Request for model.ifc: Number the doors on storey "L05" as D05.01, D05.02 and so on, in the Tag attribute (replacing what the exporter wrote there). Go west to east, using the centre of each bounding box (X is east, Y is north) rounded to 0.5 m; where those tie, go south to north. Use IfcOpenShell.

First a look at what the model holds.

```python
import ifcopenshell
import ifcopenshell.util.element
import ifcopenshell.util.placement

model = ifcopenshell.open("model.ifc")
print(model.schema)
storey = next(s for s in model.by_type("IfcBuildingStorey") if s.Name == "L05")
doors = [e for e in ifcopenshell.util.element.get_decomposition(storey) if e.is_a("IfcDoor")]
for e in sorted(doors, key=lambda e: e.id()):
    origin = ifcopenshell.util.placement.get_local_placement(e.ObjectPlacement)[:3, 3]
    print(e.id(), e.Tag, e.Name, origin.round(2) + 0.0, sep=" | ")
```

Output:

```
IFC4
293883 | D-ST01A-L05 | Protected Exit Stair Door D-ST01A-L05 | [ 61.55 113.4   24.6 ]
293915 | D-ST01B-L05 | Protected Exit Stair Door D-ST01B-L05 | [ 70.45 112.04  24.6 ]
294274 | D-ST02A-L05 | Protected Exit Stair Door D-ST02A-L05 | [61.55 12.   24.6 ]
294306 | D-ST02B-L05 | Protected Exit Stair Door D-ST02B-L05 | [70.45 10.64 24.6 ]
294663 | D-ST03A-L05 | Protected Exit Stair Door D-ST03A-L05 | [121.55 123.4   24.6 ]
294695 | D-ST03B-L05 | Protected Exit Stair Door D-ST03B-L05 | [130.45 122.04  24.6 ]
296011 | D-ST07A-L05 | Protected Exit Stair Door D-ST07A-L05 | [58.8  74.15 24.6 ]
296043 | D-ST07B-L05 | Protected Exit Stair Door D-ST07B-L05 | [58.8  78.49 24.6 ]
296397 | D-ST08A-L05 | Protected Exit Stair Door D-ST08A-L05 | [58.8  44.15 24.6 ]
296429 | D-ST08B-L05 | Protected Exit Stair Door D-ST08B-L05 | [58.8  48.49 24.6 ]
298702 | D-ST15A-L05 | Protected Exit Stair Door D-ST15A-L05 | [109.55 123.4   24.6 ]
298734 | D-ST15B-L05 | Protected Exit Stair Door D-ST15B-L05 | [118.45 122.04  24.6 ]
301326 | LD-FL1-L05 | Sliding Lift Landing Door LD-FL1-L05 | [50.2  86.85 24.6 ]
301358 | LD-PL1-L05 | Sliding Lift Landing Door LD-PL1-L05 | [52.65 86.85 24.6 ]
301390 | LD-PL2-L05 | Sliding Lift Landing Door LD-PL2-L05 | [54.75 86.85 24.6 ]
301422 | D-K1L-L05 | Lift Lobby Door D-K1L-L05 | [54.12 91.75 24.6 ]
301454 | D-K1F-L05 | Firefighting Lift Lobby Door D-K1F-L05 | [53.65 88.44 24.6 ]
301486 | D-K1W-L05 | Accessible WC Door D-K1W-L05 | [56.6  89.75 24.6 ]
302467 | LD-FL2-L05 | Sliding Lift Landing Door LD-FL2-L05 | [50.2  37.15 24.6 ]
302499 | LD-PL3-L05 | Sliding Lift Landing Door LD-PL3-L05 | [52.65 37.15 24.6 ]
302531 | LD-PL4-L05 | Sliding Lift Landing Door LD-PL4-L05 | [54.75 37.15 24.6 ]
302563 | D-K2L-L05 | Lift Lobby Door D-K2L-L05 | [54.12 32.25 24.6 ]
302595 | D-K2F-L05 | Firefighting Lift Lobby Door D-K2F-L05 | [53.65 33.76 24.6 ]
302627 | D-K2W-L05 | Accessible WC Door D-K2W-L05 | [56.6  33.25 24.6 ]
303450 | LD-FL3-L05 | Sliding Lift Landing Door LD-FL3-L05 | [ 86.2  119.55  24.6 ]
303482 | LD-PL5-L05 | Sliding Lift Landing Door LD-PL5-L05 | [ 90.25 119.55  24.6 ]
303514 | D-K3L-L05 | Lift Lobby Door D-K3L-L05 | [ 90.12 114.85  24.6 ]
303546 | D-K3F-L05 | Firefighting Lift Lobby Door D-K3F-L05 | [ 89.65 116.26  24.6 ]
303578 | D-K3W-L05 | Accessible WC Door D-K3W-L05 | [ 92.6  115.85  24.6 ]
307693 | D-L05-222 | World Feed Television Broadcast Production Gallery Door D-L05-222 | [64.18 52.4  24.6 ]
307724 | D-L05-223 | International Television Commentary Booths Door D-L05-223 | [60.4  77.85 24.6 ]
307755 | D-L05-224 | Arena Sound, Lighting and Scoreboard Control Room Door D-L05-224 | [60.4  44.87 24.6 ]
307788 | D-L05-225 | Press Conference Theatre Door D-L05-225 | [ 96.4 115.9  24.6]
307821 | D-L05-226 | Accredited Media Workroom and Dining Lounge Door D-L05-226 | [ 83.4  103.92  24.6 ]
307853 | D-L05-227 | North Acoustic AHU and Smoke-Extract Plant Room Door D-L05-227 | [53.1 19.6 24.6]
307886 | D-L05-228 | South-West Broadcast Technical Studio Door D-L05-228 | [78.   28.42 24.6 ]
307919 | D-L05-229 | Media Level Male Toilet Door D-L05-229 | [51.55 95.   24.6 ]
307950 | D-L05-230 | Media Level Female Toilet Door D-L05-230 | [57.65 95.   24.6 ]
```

```python
import ifcopenshell
import ifcopenshell.geom
import ifcopenshell.util.element
import ifcopenshell.util.shape

model = ifcopenshell.open("model.ifc")
settings = ifcopenshell.geom.settings()
settings.set("use-world-coords", True)


def centre(element):
    shape = ifcopenshell.geom.create_shape(settings, element)
    return ifcopenshell.util.shape.get_bbox_centroid(shape.geometry)


storey = next(s for s in model.by_type("IfcBuildingStorey") if s.Name == "L05")
doors = [e for e in ifcopenshell.util.element.get_decomposition(storey) if e.is_a("IfcDoor")]

# Insertion points can sit at a corner or the storey origin, so sort by the geometry (in metres).
centres = {e: centre(e) for e in doors}
doors.sort(key=lambda e: (round(centres[e][0] / 0.5), centres[e][1]))

for i, e in enumerate(doors, start=1):
    number = f"D05.{i:02d}"
    e.Tag = number
    print(e.id(), number)

model.write("model_edited.ifc")
```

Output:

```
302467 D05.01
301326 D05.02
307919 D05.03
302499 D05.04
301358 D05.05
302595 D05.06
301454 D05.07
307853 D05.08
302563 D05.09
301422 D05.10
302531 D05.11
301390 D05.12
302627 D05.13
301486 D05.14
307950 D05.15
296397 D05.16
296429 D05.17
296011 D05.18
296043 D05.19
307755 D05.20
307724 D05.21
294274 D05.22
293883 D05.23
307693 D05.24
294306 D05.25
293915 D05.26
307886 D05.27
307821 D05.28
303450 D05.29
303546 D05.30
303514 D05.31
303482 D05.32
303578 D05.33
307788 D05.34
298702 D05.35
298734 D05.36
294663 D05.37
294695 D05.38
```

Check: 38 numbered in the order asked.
